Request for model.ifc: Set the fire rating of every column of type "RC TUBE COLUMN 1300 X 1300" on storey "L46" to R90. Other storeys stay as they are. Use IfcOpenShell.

First a look at what the model holds.

```python
import ifcopenshell
import ifcopenshell.util.element

model = ifcopenshell.open("model.ifc")
print(model.schema)
storey = next(s for s in model.by_type("IfcBuildingStorey") if s.Name == "L46")
columns = [e for e in ifcopenshell.util.element.get_decomposition(storey) if e.is_a("IfcColumn")]
seen = {}
for e in columns:
    element_type = ifcopenshell.util.element.get_type(e)
    key = (element_type.Name if element_type != e and element_type else None, ifcopenshell.util.element.get_pset(e, "Pset_ColumnCommon", "FireRating"))
    seen[key] = seen.get(key, 0) + 1
for (name, value), count in sorted(seen.items(), key=str):
    print(count, "x", name, "|", value)
```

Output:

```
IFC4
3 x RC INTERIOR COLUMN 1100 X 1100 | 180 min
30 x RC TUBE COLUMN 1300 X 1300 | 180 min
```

```python
import ifcopenshell
import ifcopenshell.api.pset
import ifcopenshell.util.element

model = ifcopenshell.open("model.ifc")

storey = next(s for s in model.by_type("IfcBuildingStorey") if s.Name == "L46")
columns = [e for e in ifcopenshell.util.element.get_decomposition(storey) if e.is_a("IfcColumn")]

count = 0
for e in columns:
    element_type = ifcopenshell.util.element.get_type(e)
    if element_type in (None, e) or element_type.Name != "RC TUBE COLUMN 1300 X 1300":
        continue
    found = ifcopenshell.util.element.get_pset(e, "Pset_ColumnCommon", should_inherit=False)
    if found:
        pset = model.by_id(found["id"])
        if len(ifcopenshell.util.element.get_elements_by_pset(pset)) > 1:
            pset = ifcopenshell.api.pset.unshare_pset(model, products=[e], pset=pset)[0]
    else:
        pset = ifcopenshell.api.pset.add_pset(model, product=e, name="Pset_ColumnCommon")
    ifcopenshell.api.pset.edit_pset(model, pset=pset, properties={"FireRating": "R90"})
    count += 1

print(count, "columns updated")

model.write("model_v2.ifc")
```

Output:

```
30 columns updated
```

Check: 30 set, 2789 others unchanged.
